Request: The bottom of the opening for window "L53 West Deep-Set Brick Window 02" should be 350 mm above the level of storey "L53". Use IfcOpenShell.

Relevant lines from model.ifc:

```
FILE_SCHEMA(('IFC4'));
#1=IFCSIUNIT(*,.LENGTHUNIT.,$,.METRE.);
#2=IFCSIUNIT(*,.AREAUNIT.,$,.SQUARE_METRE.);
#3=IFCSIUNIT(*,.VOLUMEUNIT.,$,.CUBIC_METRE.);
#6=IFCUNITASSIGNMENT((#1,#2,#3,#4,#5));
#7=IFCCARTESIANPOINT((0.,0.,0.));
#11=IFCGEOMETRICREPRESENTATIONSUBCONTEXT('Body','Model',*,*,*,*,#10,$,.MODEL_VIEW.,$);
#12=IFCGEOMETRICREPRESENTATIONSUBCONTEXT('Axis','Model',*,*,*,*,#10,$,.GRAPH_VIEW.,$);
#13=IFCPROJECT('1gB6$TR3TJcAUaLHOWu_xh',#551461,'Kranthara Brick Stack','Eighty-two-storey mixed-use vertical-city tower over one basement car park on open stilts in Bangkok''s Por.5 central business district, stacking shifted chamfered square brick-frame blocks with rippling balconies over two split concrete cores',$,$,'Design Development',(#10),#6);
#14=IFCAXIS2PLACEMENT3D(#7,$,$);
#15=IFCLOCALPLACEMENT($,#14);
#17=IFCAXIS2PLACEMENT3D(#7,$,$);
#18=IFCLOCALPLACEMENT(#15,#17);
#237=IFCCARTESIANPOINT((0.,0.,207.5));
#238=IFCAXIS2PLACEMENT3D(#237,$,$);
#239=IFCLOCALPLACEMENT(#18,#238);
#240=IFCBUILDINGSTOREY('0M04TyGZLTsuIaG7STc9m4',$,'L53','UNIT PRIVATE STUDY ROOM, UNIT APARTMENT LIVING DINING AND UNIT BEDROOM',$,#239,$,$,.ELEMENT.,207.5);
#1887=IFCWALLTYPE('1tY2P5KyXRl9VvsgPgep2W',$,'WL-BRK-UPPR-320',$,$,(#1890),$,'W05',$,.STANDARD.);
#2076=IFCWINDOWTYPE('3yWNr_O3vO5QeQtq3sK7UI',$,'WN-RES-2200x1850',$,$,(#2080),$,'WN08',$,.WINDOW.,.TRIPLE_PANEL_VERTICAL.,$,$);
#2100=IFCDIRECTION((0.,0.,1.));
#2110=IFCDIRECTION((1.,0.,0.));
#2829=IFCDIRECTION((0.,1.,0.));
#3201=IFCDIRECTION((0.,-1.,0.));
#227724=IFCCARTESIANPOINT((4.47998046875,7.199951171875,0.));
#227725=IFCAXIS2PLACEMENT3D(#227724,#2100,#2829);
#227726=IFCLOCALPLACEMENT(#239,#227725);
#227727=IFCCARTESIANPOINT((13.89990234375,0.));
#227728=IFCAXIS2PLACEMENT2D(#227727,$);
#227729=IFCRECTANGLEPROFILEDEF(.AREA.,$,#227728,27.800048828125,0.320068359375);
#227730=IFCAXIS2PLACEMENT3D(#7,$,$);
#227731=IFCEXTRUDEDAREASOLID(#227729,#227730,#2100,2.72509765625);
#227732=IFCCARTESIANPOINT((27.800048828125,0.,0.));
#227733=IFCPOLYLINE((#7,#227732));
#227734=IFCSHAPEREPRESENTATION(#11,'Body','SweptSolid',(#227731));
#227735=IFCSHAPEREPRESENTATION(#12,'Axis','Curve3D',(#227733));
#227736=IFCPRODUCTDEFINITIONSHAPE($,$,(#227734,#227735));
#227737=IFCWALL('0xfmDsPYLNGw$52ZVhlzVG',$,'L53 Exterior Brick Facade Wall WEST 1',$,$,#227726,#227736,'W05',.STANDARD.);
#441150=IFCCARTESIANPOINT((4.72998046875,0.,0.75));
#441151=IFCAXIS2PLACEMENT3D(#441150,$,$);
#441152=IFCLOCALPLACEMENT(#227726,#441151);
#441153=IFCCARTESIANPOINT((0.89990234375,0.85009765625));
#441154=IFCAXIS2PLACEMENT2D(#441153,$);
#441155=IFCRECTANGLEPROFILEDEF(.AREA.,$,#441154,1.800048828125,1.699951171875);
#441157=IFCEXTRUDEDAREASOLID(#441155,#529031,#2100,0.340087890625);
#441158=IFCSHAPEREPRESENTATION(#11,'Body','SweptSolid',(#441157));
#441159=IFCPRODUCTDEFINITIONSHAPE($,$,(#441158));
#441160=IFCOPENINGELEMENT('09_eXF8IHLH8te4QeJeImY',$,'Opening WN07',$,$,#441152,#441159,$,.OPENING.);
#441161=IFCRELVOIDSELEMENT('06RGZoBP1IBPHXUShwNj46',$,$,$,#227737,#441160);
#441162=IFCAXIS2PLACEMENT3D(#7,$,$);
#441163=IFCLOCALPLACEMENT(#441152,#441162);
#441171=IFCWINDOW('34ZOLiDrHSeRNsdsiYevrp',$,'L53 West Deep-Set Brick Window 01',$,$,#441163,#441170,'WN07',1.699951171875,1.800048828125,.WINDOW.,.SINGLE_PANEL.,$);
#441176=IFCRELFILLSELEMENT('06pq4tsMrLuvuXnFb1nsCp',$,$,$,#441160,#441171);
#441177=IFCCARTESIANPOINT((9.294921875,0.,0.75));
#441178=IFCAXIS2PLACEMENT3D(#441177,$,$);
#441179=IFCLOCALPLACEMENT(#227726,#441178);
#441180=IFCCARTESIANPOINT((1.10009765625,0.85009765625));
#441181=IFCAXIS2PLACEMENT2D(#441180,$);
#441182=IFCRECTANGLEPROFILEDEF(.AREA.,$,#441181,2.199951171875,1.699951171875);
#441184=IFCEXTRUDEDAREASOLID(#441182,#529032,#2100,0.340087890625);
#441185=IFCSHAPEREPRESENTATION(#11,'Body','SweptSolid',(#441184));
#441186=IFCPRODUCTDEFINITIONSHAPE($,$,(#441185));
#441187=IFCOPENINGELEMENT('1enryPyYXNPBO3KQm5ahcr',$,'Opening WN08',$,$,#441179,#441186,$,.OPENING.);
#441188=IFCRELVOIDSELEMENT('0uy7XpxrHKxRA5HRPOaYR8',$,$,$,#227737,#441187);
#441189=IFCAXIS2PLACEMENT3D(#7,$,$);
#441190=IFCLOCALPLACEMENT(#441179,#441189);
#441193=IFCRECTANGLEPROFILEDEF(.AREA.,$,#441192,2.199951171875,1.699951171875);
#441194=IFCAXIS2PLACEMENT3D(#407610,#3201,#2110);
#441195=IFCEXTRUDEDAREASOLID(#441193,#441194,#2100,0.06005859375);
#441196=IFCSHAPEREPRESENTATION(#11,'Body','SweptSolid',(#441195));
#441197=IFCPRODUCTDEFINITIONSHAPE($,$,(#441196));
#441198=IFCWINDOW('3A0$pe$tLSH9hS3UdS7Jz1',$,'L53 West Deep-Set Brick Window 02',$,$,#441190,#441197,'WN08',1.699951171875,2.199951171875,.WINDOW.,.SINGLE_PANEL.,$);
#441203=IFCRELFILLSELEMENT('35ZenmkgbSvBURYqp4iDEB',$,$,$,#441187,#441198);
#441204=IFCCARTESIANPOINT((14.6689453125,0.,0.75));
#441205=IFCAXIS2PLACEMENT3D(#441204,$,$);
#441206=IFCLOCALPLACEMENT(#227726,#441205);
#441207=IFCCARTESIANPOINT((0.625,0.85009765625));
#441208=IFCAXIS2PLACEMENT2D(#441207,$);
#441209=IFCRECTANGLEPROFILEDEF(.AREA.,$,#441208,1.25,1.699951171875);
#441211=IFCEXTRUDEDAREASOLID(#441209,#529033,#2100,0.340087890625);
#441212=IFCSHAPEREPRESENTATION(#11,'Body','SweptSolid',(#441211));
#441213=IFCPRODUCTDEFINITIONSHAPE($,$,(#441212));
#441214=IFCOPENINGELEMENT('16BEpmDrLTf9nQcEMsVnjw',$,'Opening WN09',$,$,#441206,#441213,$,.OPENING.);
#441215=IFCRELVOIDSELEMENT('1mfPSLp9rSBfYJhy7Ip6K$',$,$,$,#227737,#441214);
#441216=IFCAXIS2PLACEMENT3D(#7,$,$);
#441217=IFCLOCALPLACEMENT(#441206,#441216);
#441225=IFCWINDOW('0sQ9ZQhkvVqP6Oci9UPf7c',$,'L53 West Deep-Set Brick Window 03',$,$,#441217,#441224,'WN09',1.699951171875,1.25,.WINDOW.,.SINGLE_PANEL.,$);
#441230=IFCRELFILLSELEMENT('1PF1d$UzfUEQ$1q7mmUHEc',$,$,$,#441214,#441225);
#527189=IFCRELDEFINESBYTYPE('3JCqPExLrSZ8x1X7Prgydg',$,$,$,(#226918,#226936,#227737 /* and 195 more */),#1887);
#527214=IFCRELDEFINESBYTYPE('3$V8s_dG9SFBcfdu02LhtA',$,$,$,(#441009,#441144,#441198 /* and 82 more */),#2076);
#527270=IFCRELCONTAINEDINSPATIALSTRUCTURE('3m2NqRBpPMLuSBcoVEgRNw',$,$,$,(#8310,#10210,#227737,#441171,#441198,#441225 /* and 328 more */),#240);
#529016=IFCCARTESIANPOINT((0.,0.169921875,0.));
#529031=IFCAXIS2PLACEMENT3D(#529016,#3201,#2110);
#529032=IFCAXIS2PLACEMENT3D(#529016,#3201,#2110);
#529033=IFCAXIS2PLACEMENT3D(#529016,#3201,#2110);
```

```python
import numpy as np
import ifcopenshell
import ifcopenshell.api.geometry
import ifcopenshell.geom
import ifcopenshell.util.element
import ifcopenshell.util.placement
import ifcopenshell.util.shape
import ifcopenshell.util.unit

model = ifcopenshell.open("model.ifc")
unit_scale = ifcopenshell.util.unit.calculate_unit_scale(model)

window = model.by_guid("3A0$pe$tLSH9hS3UdS7Jz1")
opening = window.FillsVoids[0].RelatingOpeningElement
storey = ifcopenshell.util.element.get_container(window, ifc_class="IfcBuildingStorey")
level = ifcopenshell.util.placement.get_local_placement(storey.ObjectPlacement)[2, 3]

# The opening's origin need not be at the sill, so measure its lowest point.
shape = ifcopenshell.geom.create_shape(ifcopenshell.geom.settings(), opening)
bottom = ifcopenshell.util.shape.get_shape_bottom_elevation(shape, shape.geometry) / unit_scale
dz = level + 0.35 / unit_scale - bottom

shift = np.array([0.0, 0.0, dz])
# The window is placed relative to its opening, so it follows when the opening moves.
matrix = ifcopenshell.util.placement.get_local_placement(opening.ObjectPlacement)
matrix[:3, 3] += shift
ifcopenshell.api.geometry.edit_object_placement(
    model, product=opening, matrix=matrix, is_si=False, should_transform_children=True
)

print(f"moved by {dz * unit_scale:+.3f} m")

model.write("model_edited.ifc")
```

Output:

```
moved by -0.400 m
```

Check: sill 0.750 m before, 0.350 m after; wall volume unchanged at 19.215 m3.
